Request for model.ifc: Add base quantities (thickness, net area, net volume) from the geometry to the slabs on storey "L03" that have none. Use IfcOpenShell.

First a look at what the model holds.

```python
import ifcopenshell
import ifcopenshell.util.element
import ifcopenshell.util.unit

model = ifcopenshell.open("model.ifc")
print(model.schema)
for unit_type in ("LENGTHUNIT", "AREAUNIT", "VOLUMEUNIT"):
    print(unit_type, ifcopenshell.util.unit.calculate_unit_scale(model, unit_type))
storey = next(s for s in model.by_type("IfcBuildingStorey") if s.Name == "L03")
slabs = [e for e in ifcopenshell.util.element.get_decomposition(storey) if e.is_a("IfcSlab")]
for e in sorted(slabs, key=lambda e: e.id()):
    print(e.id(), e.is_a(), e.Name, list(ifcopenshell.util.element.get_psets(e, qtos_only=True)), sep=" | ")
```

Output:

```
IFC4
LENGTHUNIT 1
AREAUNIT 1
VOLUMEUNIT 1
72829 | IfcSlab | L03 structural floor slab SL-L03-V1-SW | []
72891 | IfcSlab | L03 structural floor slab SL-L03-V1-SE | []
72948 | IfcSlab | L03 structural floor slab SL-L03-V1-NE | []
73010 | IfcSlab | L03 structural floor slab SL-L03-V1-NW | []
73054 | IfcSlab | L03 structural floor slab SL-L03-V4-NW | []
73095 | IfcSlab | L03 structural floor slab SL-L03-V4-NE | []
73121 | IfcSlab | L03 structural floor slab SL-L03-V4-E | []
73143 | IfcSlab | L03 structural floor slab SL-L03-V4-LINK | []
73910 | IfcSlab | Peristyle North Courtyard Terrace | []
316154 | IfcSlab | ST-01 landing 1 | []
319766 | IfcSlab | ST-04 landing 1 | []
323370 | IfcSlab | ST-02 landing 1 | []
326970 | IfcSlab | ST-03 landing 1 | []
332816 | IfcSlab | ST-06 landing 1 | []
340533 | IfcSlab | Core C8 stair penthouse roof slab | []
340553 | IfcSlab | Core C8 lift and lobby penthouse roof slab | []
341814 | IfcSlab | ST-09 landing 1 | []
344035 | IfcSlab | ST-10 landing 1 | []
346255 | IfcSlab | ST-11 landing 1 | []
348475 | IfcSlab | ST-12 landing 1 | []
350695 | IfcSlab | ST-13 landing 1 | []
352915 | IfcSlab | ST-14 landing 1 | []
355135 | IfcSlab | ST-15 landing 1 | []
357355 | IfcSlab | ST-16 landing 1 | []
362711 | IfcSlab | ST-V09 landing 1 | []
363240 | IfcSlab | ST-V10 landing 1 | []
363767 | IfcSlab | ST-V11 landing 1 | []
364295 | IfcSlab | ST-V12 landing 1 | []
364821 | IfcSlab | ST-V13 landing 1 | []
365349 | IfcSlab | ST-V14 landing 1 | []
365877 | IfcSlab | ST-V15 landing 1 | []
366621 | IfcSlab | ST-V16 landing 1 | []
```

```python
import ifcopenshell
import ifcopenshell.api.pset
import ifcopenshell.geom
import ifcopenshell.util.element
import ifcopenshell.util.shape
import ifcopenshell.util.unit

model = ifcopenshell.open("model.ifc")
unit_scale = ifcopenshell.util.unit.calculate_unit_scale(model)
area_scale = ifcopenshell.util.unit.calculate_unit_scale(model, "AREAUNIT")
volume_scale = ifcopenshell.util.unit.calculate_unit_scale(model, "VOLUMEUNIT")
settings = ifcopenshell.geom.settings()

storey = next(s for s in model.by_type("IfcBuildingStorey") if s.Name == "L03")
slabs = [e for e in ifcopenshell.util.element.get_decomposition(storey) if e.is_a("IfcSlab")]

for e in sorted(slabs, key=lambda e: e.id()):
    if ifcopenshell.util.element.get_psets(e, qtos_only=True, should_inherit=False):
        continue
    # Geometry comes back in metres, in the element's own axes.
    shape = ifcopenshell.geom.create_shape(settings, e)
    values = {
        "Width": ifcopenshell.util.shape.get_z(shape.geometry) / unit_scale,
        "NetArea": ifcopenshell.util.shape.get_footprint_area(shape.geometry) / area_scale,
        "NetVolume": ifcopenshell.util.shape.get_volume(shape.geometry) / volume_scale,
    }
    qto = ifcopenshell.api.pset.add_qto(model, product=e, name="Qto_SlabBaseQuantities")
    ifcopenshell.api.pset.edit_qto(model, qto=qto, properties=values)
    print(e.id(), {k: round(v, 3) for k, v in values.items()})

model.write("model_rev.ifc")
```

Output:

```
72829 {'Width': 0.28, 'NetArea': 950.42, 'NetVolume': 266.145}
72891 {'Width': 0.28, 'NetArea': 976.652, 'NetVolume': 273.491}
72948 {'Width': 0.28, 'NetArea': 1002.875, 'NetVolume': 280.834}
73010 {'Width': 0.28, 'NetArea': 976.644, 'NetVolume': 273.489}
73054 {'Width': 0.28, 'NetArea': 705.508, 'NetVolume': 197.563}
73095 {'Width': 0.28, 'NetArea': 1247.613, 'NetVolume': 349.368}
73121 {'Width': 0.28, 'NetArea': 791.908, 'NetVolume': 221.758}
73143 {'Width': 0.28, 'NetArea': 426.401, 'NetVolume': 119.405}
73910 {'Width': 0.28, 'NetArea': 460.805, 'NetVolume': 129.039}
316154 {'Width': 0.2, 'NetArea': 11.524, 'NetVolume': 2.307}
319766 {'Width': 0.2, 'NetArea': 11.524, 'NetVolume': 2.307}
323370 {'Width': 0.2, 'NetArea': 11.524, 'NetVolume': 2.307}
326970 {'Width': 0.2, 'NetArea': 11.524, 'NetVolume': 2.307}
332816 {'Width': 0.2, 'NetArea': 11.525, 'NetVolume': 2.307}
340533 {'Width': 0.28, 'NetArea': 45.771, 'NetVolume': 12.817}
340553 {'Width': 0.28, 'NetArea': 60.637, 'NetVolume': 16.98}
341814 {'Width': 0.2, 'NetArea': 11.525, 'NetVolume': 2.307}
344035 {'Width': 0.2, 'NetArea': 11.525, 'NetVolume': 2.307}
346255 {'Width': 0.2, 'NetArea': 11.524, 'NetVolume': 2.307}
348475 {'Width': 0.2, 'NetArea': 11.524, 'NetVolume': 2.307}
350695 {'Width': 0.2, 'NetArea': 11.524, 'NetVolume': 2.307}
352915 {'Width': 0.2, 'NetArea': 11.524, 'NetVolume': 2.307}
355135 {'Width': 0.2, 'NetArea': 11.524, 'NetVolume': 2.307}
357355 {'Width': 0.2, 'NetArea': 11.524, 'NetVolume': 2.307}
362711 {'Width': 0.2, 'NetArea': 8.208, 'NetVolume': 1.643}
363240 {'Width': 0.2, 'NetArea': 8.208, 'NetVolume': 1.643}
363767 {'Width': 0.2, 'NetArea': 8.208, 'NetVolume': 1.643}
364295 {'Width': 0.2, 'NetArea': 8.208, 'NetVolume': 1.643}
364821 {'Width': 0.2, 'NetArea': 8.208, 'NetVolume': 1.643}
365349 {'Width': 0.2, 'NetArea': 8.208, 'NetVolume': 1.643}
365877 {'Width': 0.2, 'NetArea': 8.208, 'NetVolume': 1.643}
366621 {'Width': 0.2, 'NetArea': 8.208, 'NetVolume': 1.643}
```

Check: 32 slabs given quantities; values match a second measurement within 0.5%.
